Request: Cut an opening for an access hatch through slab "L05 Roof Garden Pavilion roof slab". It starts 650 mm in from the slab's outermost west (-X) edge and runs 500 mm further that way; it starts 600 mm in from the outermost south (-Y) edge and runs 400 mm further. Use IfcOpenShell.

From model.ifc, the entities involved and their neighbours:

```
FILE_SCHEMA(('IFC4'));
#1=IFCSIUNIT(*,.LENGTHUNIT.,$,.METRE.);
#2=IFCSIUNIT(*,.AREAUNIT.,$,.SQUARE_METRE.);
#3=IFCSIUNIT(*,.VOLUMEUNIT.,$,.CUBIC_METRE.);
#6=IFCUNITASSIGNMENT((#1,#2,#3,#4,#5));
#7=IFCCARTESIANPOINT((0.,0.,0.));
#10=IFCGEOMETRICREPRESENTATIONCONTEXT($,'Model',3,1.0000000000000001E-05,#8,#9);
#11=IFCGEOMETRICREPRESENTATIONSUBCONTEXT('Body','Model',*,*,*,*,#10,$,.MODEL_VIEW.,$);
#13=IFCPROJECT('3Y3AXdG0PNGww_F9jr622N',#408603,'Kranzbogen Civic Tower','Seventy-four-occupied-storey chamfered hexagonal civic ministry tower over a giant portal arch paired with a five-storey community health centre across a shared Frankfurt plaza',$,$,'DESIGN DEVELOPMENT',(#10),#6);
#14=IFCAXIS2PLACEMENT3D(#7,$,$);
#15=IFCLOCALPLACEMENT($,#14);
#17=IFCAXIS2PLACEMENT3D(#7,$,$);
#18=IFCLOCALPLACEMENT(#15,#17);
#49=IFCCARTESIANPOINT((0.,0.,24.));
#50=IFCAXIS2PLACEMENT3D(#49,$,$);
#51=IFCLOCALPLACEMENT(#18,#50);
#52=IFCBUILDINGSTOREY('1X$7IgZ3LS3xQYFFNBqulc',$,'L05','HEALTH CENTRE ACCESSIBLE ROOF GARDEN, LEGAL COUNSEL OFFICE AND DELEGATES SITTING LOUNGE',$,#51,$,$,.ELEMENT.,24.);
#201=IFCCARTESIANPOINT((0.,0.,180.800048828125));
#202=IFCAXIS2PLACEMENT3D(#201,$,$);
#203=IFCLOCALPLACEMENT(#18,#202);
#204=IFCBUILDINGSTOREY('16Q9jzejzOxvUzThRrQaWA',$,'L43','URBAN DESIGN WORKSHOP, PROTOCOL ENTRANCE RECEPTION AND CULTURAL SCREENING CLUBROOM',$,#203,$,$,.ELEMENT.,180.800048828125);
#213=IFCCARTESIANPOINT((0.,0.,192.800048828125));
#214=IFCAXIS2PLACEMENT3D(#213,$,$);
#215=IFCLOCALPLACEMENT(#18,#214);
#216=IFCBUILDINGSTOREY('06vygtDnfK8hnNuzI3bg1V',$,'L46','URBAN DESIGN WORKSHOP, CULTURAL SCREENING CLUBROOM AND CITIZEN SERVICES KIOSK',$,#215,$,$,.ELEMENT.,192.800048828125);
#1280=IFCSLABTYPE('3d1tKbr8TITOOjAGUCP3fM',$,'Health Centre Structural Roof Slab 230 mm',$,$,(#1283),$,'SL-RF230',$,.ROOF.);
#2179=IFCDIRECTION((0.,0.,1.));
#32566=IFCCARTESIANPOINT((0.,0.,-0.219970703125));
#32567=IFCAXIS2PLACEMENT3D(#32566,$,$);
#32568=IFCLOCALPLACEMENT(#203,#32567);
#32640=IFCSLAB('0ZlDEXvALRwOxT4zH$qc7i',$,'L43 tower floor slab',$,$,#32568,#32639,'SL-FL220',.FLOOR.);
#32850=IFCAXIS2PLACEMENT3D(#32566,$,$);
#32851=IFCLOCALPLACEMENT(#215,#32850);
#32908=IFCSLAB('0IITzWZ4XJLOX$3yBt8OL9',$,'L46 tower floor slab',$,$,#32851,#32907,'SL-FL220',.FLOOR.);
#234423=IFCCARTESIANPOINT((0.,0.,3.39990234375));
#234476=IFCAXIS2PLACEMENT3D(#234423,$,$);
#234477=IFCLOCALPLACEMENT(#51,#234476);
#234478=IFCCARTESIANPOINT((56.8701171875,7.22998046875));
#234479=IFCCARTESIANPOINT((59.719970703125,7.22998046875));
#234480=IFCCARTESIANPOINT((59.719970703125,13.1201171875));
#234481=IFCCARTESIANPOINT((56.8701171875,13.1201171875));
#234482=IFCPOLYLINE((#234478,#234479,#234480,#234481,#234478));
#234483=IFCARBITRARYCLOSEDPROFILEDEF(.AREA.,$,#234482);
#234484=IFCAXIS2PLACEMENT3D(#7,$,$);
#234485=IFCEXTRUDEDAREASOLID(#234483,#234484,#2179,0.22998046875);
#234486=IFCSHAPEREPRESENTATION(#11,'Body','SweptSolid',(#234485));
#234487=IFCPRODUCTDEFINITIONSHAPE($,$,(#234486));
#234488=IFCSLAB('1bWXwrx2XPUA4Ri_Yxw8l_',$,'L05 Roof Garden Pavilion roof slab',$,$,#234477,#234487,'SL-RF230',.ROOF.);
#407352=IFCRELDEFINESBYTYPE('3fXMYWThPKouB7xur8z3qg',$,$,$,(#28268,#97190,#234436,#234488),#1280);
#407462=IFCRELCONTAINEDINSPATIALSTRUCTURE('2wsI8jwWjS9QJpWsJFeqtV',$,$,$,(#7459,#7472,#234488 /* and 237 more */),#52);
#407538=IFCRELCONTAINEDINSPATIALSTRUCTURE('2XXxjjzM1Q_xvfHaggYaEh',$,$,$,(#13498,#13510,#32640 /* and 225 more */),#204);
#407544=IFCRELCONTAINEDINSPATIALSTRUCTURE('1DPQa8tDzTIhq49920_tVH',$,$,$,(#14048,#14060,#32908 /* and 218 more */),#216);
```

```python
import numpy as np
import ifcopenshell
import ifcopenshell.api.feature
import ifcopenshell.api.geometry
import ifcopenshell.api.root
import ifcopenshell.geom
import ifcopenshell.util.placement
import ifcopenshell.util.representation
import ifcopenshell.util.shape
import ifcopenshell.util.unit

model = ifcopenshell.open("model.ifc")
unit_scale = ifcopenshell.util.unit.calculate_unit_scale(model)
settings = ifcopenshell.geom.settings()


def volume(element):
    """Net volume in cubic metres, openings subtracted."""
    shape = ifcopenshell.geom.create_shape(settings, element)
    return ifcopenshell.util.shape.get_volume(shape.geometry)


slab = model.by_guid("1bWXwrx2XPUA4Ri_Yxw8l_")
before = volume(slab)

# Extent in the slab's own axes, in metres. The edges named are its -X and -Y sides.
slab_shape = ifcopenshell.geom.create_shape(settings, slab)
vertices = ifcopenshell.util.shape.get_vertices(slab_shape.geometry)
x_min, y_min, bottom = vertices.min(axis=0)
top = vertices[:, 2].max()

opening = ifcopenshell.api.root.create_entity(model, ifc_class="IfcOpeningElement", name="Access hatch opening", predefined_type="OPENING")
context = ifcopenshell.util.representation.get_context(model, "Model", "Body", "MODEL_VIEW")
width, depth = 0.5, 0.4
outline = [(0.0, 0.0), (width, 0.0), (width, depth), (0.0, depth), (0.0, 0.0)]
# Overshoot both faces by 50 mm so the cut is clean.
shape = ifcopenshell.api.geometry.add_slab_representation(
    model, context=context, depth=top - bottom + 0.1, polyline=outline
)
ifcopenshell.api.geometry.assign_representation(model, product=opening, representation=shape)

matrix = ifcopenshell.util.placement.get_local_placement(slab.ObjectPlacement)
matrix[:, 3] = matrix @ np.append(np.array([x_min + 0.65, y_min + 0.6, bottom - 0.05]) / unit_scale, 1.0)
ifcopenshell.api.geometry.edit_object_placement(model, product=opening, matrix=matrix, is_si=False)
ifcopenshell.api.feature.add_feature(model, feature=opening, element=slab)

after = volume(slab)

print(f"slab volume {before:.3f} -> {after:.3f} m3")

model.write("model-out.ifc")
```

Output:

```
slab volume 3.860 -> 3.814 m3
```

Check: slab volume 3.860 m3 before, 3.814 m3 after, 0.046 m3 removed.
